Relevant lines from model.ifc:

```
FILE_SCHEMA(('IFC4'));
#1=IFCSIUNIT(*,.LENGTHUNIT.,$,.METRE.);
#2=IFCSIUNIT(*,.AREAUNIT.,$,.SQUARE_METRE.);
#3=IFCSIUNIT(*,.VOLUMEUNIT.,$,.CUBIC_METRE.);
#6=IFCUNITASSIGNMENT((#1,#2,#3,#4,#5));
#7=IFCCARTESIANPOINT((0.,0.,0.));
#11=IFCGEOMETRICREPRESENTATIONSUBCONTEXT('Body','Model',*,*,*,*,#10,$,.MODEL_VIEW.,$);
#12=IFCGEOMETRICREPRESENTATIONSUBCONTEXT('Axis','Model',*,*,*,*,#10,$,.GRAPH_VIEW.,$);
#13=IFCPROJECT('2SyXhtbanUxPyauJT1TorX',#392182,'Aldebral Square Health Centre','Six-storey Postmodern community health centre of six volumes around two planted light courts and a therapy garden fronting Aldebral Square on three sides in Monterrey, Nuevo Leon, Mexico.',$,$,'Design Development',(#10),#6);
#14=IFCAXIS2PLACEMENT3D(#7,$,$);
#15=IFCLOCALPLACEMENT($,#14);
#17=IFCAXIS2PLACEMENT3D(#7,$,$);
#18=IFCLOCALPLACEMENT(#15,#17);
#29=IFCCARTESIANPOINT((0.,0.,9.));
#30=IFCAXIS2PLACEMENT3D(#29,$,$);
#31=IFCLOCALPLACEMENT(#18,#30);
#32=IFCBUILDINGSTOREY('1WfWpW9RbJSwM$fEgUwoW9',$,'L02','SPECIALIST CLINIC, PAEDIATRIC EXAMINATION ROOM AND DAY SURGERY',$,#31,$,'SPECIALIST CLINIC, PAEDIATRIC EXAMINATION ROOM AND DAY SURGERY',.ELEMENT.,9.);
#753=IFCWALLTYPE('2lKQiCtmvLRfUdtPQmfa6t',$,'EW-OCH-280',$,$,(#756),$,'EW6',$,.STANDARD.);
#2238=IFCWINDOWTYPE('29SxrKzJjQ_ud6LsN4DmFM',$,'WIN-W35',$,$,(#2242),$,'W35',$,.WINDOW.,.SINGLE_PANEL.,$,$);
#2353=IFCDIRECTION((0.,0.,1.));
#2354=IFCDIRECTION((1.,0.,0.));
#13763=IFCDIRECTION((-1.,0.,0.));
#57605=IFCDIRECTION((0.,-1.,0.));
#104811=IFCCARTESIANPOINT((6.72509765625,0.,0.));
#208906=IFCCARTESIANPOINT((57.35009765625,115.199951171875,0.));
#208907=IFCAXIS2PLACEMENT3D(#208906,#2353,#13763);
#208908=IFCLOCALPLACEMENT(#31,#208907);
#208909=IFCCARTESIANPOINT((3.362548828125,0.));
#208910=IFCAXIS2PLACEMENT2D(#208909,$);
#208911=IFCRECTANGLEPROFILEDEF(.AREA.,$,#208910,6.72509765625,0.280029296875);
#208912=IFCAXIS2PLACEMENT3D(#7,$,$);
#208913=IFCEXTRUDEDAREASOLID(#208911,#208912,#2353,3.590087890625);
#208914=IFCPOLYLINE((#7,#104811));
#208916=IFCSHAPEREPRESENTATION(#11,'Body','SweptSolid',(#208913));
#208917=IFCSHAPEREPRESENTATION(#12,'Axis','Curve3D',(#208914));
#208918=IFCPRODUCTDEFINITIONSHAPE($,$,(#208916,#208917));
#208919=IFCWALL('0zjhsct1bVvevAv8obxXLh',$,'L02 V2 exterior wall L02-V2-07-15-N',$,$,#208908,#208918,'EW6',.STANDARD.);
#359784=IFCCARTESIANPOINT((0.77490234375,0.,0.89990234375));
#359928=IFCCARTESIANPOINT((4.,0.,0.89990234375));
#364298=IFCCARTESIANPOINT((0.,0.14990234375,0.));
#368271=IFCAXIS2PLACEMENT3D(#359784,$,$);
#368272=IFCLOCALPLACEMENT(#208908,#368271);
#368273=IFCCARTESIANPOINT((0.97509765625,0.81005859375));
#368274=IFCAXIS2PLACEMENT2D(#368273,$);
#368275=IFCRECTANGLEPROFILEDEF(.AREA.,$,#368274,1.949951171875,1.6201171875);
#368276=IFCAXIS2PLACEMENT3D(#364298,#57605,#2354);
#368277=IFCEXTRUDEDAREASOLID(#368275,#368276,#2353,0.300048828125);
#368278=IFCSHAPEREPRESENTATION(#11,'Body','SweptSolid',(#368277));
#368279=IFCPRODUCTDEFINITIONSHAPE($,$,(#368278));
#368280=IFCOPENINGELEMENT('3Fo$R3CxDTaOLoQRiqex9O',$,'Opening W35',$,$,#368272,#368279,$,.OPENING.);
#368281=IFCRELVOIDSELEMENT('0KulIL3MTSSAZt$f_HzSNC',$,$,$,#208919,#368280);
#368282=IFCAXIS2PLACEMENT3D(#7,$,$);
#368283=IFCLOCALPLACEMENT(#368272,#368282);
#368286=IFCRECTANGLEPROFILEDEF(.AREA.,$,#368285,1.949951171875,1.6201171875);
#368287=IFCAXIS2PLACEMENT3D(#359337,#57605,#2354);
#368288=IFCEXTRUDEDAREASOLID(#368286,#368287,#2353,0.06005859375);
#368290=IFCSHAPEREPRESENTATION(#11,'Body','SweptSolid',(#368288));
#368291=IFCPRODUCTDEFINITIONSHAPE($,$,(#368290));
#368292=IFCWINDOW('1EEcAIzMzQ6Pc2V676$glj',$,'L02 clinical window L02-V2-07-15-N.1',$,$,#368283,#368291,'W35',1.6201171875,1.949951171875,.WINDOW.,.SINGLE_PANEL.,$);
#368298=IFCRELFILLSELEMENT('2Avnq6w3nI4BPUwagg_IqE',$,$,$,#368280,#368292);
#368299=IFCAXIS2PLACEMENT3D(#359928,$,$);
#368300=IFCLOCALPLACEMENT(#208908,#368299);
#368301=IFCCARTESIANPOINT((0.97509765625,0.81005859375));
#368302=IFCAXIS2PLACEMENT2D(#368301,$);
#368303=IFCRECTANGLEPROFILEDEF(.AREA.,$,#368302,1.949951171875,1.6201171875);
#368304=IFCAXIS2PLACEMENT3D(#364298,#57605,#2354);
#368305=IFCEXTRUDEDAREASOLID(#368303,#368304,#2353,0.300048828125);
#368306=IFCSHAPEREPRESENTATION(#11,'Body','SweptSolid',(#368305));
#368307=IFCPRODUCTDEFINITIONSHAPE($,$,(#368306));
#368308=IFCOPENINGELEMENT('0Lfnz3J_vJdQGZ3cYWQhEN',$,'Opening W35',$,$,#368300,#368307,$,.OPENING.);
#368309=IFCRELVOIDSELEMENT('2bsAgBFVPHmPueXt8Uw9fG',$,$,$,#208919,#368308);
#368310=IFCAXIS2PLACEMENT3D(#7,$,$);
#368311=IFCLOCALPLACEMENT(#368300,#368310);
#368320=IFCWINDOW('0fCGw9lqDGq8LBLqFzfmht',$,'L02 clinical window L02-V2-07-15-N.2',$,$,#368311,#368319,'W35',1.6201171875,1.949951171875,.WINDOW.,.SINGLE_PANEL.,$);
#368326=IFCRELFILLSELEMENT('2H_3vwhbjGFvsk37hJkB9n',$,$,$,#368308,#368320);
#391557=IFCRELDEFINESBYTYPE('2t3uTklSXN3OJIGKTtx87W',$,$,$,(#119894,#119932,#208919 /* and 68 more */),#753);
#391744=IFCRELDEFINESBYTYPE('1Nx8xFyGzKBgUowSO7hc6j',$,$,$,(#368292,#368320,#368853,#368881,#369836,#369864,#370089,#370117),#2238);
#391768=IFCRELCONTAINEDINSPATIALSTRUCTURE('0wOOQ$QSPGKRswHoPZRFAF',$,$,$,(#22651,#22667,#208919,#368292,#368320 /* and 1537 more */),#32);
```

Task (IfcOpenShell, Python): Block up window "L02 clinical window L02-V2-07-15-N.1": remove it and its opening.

```python
import ifcopenshell
import ifcopenshell.api.feature
import ifcopenshell.api.root
import ifcopenshell.geom
import ifcopenshell.util.shape

model = ifcopenshell.open("model.ifc")
settings = ifcopenshell.geom.settings()


def volume(element):
    """Net volume in cubic metres, openings subtracted."""
    shape = ifcopenshell.geom.create_shape(settings, element)
    return ifcopenshell.util.shape.get_volume(shape.geometry)


window = model.by_guid("1EEcAIzMzQ6Pc2V676$glj")
opening = window.FillsVoids[0].RelatingOpeningElement
wall = opening.VoidsElements[0].RelatingBuildingElement
before = volume(wall)

ifcopenshell.api.root.remove_product(model, product=window)
ifcopenshell.api.feature.remove_feature(model, feature=opening)

after = volume(wall)

print(f"wall volume {before:.3f} -> {after:.3f} m3")

model.write("model_updated.ifc")
```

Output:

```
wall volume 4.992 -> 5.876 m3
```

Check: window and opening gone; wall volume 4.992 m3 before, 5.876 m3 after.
